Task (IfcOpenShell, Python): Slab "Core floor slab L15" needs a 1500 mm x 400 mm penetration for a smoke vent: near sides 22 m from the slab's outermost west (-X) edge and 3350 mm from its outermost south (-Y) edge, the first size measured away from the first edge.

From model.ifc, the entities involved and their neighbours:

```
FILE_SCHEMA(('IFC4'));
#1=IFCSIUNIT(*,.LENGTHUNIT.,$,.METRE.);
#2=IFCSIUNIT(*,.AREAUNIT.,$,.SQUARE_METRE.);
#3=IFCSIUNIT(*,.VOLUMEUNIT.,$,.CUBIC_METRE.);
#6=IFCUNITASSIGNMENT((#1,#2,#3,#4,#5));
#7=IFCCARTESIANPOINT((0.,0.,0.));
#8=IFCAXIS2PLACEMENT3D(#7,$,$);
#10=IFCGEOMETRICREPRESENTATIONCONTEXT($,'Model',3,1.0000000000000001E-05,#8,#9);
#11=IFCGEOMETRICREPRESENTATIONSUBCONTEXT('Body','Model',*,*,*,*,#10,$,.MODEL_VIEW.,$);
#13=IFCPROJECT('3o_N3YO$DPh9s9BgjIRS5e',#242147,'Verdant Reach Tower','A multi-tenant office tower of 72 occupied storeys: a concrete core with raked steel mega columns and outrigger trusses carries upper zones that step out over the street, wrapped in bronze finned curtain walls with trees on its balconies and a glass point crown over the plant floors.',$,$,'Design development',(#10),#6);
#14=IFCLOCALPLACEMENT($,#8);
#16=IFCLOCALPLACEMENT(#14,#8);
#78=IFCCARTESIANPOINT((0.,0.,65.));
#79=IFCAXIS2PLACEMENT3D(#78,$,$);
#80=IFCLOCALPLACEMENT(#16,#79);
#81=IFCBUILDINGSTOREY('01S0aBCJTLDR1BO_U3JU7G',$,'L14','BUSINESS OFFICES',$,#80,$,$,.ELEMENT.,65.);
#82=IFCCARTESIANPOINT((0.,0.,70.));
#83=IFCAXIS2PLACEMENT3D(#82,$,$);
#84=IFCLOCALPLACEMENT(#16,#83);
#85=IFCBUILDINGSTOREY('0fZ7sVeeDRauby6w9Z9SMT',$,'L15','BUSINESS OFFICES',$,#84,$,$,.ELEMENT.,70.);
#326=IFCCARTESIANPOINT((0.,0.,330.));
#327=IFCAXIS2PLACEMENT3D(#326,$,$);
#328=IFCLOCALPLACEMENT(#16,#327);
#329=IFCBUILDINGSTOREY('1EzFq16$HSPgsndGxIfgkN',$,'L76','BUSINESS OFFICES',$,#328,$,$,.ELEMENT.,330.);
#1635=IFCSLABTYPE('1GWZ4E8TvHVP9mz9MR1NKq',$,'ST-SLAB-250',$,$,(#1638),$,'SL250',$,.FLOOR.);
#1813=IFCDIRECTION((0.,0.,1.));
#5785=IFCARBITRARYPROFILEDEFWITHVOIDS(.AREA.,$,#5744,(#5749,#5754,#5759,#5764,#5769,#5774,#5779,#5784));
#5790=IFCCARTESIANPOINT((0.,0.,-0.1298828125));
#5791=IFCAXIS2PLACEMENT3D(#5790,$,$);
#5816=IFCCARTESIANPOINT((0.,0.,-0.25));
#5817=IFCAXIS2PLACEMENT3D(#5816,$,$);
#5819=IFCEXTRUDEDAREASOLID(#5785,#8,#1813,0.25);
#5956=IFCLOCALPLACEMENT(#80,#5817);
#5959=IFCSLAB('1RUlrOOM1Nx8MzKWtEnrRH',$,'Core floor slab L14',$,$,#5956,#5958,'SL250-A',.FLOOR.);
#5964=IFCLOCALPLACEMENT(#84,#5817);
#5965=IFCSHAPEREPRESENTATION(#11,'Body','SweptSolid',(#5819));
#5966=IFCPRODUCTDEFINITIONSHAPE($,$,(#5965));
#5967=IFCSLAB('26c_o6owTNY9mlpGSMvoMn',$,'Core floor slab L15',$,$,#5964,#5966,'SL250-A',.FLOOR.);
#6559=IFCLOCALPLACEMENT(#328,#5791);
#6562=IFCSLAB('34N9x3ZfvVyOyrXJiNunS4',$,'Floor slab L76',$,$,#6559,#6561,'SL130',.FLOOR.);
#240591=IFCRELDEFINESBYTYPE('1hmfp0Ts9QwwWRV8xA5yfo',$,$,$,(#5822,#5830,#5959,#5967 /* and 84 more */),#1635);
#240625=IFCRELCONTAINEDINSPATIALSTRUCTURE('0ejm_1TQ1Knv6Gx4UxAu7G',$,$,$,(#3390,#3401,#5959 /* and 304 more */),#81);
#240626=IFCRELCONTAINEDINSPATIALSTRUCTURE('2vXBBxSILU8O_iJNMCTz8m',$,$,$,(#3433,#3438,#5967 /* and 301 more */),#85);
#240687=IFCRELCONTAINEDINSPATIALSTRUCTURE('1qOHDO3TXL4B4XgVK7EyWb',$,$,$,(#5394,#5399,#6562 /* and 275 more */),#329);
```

```python
import numpy as np
import ifcopenshell
import ifcopenshell.api.feature
import ifcopenshell.api.geometry
import ifcopenshell.api.root
import ifcopenshell.geom
import ifcopenshell.util.placement
import ifcopenshell.util.representation
import ifcopenshell.util.shape
import ifcopenshell.util.unit

model = ifcopenshell.open("model.ifc")
unit_scale = ifcopenshell.util.unit.calculate_unit_scale(model)
settings = ifcopenshell.geom.settings()


def volume(element):
    """Net volume in cubic metres, openings subtracted."""
    shape = ifcopenshell.geom.create_shape(settings, element)
    return ifcopenshell.util.shape.get_volume(shape.geometry)


slab = model.by_guid("26c_o6owTNY9mlpGSMvoMn")
before = volume(slab)

# Extent in the slab's own axes, in metres. The edges named are its -X and -Y sides.
slab_shape = ifcopenshell.geom.create_shape(settings, slab)
vertices = ifcopenshell.util.shape.get_vertices(slab_shape.geometry)
x_min, y_min, bottom = vertices.min(axis=0)
top = vertices[:, 2].max()

opening = ifcopenshell.api.root.create_entity(model, ifc_class="IfcOpeningElement", name="Smoke vent opening", predefined_type="OPENING")
context = ifcopenshell.util.representation.get_context(model, "Model", "Body", "MODEL_VIEW")
width, depth = 1.5, 0.4
outline = [(0.0, 0.0), (width, 0.0), (width, depth), (0.0, depth), (0.0, 0.0)]
# Overshoot both faces by 50 mm so the cut is clean.
shape = ifcopenshell.api.geometry.add_slab_representation(
    model, context=context, depth=top - bottom + 0.1, polyline=outline
)
ifcopenshell.api.geometry.assign_representation(model, product=opening, representation=shape)

matrix = ifcopenshell.util.placement.get_local_placement(slab.ObjectPlacement)
matrix[:, 3] = matrix @ np.append(np.array([x_min + 22, y_min + 3.35, bottom - 0.05]) / unit_scale, 1.0)
ifcopenshell.api.geometry.edit_object_placement(model, product=opening, matrix=matrix, is_si=False)
ifcopenshell.api.feature.add_feature(model, feature=opening, element=slab)

after = volume(slab)

print(f"slab volume {before:.3f} -> {after:.3f} m3")

model.write("model_edited.ifc")
```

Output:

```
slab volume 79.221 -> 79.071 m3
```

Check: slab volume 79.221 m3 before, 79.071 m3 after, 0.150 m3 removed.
